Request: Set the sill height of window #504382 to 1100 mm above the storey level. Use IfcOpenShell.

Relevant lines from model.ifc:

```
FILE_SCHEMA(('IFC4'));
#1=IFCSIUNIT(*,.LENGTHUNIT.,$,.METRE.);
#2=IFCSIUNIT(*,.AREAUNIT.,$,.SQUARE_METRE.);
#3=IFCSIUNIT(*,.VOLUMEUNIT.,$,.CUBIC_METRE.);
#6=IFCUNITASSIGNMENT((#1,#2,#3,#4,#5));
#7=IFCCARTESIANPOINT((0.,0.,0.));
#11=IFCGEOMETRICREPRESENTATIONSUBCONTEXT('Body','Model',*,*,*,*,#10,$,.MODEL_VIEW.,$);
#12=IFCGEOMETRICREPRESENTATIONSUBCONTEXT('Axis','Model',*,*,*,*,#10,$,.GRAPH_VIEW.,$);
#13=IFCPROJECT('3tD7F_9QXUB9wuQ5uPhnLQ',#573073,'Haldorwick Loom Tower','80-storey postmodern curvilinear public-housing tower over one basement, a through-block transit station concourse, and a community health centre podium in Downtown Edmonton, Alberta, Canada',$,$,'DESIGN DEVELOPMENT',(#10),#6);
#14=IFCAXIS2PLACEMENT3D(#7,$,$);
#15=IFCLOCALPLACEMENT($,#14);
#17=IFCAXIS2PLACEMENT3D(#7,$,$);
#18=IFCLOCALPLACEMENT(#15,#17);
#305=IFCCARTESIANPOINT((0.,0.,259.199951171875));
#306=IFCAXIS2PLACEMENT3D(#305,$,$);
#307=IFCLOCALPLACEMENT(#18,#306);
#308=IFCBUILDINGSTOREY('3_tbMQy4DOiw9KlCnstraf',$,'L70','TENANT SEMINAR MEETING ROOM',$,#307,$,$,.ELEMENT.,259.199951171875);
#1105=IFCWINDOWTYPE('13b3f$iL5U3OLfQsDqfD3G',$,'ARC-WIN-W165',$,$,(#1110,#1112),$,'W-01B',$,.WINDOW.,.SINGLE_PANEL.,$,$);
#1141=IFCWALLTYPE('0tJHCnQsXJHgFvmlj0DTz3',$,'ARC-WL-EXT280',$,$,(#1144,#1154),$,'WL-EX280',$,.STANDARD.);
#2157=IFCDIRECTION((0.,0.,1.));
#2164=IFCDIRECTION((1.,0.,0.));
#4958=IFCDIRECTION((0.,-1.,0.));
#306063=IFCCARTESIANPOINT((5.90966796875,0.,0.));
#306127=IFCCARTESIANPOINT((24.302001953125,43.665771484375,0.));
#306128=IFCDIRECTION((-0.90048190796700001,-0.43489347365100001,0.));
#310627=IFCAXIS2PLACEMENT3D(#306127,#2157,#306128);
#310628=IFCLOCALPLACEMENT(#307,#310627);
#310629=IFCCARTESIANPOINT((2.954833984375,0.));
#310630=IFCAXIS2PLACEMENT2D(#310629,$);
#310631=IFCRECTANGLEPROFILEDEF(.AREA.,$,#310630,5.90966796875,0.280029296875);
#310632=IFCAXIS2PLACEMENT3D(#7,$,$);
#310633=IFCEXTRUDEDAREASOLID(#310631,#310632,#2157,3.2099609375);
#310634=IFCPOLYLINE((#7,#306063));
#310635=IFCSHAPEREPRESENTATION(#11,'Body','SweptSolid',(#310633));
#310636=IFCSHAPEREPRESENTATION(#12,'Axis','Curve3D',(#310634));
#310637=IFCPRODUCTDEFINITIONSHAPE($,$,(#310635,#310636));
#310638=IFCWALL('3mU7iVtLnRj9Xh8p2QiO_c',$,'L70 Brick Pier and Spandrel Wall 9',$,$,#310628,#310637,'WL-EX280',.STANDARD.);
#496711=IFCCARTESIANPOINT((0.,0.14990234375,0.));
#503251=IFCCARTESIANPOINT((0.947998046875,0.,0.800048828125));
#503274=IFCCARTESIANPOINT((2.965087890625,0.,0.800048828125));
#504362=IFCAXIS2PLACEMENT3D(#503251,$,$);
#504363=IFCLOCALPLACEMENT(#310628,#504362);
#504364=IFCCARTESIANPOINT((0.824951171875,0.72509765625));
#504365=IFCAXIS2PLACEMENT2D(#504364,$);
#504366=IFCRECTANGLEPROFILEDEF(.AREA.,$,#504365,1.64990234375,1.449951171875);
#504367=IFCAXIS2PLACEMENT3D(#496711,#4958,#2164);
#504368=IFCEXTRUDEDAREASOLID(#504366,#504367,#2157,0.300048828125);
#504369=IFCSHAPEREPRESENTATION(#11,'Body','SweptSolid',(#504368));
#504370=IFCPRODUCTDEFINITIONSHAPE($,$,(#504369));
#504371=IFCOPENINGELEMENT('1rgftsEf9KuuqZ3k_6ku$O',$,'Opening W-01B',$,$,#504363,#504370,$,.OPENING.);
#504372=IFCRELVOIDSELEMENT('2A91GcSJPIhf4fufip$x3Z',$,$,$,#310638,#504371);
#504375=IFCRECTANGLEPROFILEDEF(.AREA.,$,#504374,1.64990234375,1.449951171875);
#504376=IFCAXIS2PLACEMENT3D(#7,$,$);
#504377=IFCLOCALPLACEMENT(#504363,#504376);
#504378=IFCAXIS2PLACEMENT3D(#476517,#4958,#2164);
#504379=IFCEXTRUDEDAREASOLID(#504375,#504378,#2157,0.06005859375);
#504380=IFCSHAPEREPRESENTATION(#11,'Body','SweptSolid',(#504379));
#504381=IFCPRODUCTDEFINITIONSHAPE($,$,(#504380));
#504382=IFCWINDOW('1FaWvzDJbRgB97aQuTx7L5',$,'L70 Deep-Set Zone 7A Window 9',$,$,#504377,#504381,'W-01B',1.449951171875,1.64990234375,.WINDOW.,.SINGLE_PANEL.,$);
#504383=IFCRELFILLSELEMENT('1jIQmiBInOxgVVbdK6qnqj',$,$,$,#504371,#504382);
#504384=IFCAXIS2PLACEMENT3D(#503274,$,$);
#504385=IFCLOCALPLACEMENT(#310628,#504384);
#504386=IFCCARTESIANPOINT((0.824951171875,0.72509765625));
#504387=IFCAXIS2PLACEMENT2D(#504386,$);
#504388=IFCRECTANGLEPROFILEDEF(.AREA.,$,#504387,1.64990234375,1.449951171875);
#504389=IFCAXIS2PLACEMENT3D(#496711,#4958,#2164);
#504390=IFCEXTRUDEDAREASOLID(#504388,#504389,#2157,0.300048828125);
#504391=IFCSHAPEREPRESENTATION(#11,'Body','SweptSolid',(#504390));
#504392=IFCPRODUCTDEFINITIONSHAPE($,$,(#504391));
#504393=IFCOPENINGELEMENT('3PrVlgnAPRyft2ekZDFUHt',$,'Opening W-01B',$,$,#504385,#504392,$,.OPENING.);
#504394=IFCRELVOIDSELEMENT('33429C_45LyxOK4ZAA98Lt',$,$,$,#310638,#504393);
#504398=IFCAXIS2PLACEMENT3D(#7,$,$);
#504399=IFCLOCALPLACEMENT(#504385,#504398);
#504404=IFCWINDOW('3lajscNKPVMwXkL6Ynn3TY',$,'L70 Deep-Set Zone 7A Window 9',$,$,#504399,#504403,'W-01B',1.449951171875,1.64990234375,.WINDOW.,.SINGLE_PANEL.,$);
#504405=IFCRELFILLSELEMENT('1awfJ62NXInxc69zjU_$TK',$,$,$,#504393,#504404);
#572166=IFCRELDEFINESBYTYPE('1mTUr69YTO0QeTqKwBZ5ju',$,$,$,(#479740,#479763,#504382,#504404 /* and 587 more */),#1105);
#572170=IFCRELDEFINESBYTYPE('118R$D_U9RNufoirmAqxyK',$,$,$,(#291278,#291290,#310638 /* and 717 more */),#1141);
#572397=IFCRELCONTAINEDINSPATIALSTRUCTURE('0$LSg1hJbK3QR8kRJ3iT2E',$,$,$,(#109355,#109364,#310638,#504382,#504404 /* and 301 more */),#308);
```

```python
import numpy as np
import ifcopenshell
import ifcopenshell.api.geometry
import ifcopenshell.geom
import ifcopenshell.util.element
import ifcopenshell.util.placement
import ifcopenshell.util.shape
import ifcopenshell.util.unit

model = ifcopenshell.open("model.ifc")
unit_scale = ifcopenshell.util.unit.calculate_unit_scale(model)

window = model.by_id(504382)
opening = window.FillsVoids[0].RelatingOpeningElement
storey = ifcopenshell.util.element.get_container(window, ifc_class="IfcBuildingStorey")
level = ifcopenshell.util.placement.get_local_placement(storey.ObjectPlacement)[2, 3]

# The opening's origin need not be at the sill, so measure its lowest point.
shape = ifcopenshell.geom.create_shape(ifcopenshell.geom.settings(), opening)
bottom = ifcopenshell.util.shape.get_shape_bottom_elevation(shape, shape.geometry) / unit_scale
dz = level + 1.1 / unit_scale - bottom

shift = np.array([0.0, 0.0, dz])
# The window is placed relative to its opening, so it follows when the opening moves.
matrix = ifcopenshell.util.placement.get_local_placement(opening.ObjectPlacement)
matrix[:3, 3] += shift
ifcopenshell.api.geometry.edit_object_placement(
    model, product=opening, matrix=matrix, is_si=False, should_transform_children=True
)

print(f"moved by {dz * unit_scale:+.3f} m")

model.write("model-out.ifc")
```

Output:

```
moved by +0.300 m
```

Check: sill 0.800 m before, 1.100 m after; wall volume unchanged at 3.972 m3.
